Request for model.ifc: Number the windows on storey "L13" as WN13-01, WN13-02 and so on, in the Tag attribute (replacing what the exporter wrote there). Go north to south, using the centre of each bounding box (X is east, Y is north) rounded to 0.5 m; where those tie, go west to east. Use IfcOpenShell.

First a look at what the model holds.

```python
import ifcopenshell
import ifcopenshell.util.element
import ifcopenshell.util.placement

model = ifcopenshell.open("model.ifc")
print(model.schema)
storey = next(s for s in model.by_type("IfcBuildingStorey") if s.Name == "L13")
windows = [e for e in ifcopenshell.util.element.get_decomposition(storey) if e.is_a("IfcWindow")]
for e in sorted(windows, key=lambda e: e.id()):
    origin = ifcopenshell.util.placement.get_local_placement(e.ObjectPlacement)[:3, 3]
    print(e.id(), e.Tag, e.Name, origin.round(2) + 0.0, sep=" | ")
```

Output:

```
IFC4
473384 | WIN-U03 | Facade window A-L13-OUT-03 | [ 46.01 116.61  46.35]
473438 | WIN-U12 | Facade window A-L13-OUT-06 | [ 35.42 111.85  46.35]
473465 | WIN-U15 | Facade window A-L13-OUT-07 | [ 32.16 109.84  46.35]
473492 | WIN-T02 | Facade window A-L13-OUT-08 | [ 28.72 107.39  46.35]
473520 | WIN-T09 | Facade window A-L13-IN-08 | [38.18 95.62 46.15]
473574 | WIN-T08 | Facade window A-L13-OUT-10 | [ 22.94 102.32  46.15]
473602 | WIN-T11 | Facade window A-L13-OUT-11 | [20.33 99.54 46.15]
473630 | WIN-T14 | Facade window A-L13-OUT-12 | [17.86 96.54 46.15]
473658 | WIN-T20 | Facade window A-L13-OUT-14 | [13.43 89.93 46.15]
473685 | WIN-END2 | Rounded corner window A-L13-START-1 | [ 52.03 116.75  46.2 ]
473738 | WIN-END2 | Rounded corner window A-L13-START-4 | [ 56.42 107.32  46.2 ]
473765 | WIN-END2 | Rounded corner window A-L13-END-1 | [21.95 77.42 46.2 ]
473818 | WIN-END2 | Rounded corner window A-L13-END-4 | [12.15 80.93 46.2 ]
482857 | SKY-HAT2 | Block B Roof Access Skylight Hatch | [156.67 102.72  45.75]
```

```python
import ifcopenshell
import ifcopenshell.geom
import ifcopenshell.util.element
import ifcopenshell.util.shape

model = ifcopenshell.open("model.ifc")
settings = ifcopenshell.geom.settings()
settings.set("use-world-coords", True)


def centre(element):
    shape = ifcopenshell.geom.create_shape(settings, element)
    return ifcopenshell.util.shape.get_bbox_centroid(shape.geometry)


storey = next(s for s in model.by_type("IfcBuildingStorey") if s.Name == "L13")
windows = [e for e in ifcopenshell.util.element.get_decomposition(storey) if e.is_a("IfcWindow")]

# Insertion points can sit at a corner or the storey origin, so sort by the geometry (in metres).
centres = {e: centre(e) for e in windows}
windows.sort(key=lambda e: (-round(centres[e][1] / 0.5), centres[e][0]))

for i, e in enumerate(windows, start=1):
    number = f"WN13-{i:02d}"
    e.Tag = number
    print(e.id(), number)

model.write("model_rev.ifc")
```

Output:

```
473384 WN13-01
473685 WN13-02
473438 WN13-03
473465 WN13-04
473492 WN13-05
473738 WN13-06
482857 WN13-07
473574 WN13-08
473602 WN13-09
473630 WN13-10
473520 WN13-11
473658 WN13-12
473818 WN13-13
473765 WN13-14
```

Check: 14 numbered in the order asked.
